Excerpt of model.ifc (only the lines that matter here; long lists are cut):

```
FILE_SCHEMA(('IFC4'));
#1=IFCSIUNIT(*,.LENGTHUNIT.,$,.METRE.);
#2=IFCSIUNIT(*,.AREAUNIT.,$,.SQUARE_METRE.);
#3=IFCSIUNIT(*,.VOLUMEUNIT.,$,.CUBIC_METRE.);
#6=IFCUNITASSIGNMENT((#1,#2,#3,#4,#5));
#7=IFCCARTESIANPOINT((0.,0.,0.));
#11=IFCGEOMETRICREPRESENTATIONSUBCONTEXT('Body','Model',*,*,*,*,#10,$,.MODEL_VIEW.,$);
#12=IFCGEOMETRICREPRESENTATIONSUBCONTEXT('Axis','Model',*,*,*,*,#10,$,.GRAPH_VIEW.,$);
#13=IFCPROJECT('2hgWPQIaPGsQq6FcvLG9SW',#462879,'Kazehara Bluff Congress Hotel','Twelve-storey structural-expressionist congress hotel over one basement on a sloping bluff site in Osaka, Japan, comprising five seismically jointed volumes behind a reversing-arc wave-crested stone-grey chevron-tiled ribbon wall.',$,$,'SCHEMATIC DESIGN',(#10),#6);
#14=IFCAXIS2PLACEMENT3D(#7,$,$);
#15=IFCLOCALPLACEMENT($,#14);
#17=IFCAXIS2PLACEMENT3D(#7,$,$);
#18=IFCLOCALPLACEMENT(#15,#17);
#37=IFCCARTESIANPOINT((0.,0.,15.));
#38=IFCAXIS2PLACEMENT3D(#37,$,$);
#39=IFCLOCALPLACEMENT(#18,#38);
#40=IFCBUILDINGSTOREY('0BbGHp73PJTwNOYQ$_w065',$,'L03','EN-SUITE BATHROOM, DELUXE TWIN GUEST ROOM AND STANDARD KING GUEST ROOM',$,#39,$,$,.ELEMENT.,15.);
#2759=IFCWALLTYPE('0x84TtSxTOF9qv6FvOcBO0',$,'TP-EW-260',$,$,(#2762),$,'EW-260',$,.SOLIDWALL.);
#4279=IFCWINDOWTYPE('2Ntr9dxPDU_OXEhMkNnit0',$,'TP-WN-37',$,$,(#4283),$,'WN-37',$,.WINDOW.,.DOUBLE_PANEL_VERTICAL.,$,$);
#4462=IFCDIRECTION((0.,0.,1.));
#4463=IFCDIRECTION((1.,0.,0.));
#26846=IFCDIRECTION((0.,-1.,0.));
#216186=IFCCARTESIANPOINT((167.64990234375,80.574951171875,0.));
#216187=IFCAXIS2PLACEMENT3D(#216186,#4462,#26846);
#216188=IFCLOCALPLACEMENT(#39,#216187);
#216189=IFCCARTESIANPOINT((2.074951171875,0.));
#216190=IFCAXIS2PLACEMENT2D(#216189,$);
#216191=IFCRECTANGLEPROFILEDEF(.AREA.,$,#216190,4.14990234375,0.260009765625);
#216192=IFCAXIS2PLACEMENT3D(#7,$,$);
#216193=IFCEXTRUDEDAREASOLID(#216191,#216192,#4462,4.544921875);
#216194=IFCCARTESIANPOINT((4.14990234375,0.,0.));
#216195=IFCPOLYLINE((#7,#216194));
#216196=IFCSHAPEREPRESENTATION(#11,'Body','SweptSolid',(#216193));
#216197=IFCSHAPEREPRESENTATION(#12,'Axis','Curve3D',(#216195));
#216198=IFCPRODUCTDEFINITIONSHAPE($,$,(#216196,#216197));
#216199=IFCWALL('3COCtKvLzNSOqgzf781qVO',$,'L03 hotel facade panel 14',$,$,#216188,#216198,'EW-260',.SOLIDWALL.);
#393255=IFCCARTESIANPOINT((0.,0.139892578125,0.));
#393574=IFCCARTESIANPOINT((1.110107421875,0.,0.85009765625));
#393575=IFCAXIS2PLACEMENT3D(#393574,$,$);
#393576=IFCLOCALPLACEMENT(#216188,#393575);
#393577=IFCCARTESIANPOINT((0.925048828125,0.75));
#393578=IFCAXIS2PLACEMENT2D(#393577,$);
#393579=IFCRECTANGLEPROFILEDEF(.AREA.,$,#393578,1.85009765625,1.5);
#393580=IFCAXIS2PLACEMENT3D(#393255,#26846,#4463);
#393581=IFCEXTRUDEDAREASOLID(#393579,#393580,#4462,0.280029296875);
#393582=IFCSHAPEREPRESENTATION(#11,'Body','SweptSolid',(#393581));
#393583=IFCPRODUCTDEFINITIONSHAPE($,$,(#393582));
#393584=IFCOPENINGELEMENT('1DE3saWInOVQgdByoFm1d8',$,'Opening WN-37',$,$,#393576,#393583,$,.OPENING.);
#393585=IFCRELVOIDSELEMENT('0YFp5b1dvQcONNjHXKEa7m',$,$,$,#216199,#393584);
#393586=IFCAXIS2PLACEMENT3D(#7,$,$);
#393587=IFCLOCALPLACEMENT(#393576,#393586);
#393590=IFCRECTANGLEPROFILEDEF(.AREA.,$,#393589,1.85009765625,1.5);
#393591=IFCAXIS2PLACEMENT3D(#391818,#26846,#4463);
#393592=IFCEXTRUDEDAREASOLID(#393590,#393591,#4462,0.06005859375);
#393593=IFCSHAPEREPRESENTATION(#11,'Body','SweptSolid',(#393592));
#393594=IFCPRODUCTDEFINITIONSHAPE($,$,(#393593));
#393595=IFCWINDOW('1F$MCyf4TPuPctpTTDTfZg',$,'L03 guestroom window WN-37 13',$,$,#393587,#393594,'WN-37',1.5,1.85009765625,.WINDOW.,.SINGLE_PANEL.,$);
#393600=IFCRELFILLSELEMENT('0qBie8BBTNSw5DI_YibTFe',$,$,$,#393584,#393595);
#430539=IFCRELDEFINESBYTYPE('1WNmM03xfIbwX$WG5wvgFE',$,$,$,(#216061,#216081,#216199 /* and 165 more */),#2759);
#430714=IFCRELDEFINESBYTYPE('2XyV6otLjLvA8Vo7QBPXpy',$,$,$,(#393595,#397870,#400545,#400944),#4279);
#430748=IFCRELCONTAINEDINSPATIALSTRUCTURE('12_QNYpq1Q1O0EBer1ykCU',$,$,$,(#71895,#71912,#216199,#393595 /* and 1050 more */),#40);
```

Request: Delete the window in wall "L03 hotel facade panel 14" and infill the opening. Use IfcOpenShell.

```python
import ifcopenshell
import ifcopenshell.api.feature
import ifcopenshell.api.root
import ifcopenshell.geom
import ifcopenshell.util.shape

model = ifcopenshell.open("model.ifc")
settings = ifcopenshell.geom.settings()


def volume(element):
    """Net volume in cubic metres, openings subtracted."""
    shape = ifcopenshell.geom.create_shape(settings, element)
    return ifcopenshell.util.shape.get_volume(shape.geometry)


window = model.by_id(393595)
opening = window.FillsVoids[0].RelatingOpeningElement
wall = opening.VoidsElements[0].RelatingBuildingElement
before = volume(wall)

ifcopenshell.api.root.remove_product(model, product=window)
ifcopenshell.api.feature.remove_feature(model, feature=opening)

after = volume(wall)

print(f"wall volume {before:.3f} -> {after:.3f} m3")

model.write("model_rev.ifc")
```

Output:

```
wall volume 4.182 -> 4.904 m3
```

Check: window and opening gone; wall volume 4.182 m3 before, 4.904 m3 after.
